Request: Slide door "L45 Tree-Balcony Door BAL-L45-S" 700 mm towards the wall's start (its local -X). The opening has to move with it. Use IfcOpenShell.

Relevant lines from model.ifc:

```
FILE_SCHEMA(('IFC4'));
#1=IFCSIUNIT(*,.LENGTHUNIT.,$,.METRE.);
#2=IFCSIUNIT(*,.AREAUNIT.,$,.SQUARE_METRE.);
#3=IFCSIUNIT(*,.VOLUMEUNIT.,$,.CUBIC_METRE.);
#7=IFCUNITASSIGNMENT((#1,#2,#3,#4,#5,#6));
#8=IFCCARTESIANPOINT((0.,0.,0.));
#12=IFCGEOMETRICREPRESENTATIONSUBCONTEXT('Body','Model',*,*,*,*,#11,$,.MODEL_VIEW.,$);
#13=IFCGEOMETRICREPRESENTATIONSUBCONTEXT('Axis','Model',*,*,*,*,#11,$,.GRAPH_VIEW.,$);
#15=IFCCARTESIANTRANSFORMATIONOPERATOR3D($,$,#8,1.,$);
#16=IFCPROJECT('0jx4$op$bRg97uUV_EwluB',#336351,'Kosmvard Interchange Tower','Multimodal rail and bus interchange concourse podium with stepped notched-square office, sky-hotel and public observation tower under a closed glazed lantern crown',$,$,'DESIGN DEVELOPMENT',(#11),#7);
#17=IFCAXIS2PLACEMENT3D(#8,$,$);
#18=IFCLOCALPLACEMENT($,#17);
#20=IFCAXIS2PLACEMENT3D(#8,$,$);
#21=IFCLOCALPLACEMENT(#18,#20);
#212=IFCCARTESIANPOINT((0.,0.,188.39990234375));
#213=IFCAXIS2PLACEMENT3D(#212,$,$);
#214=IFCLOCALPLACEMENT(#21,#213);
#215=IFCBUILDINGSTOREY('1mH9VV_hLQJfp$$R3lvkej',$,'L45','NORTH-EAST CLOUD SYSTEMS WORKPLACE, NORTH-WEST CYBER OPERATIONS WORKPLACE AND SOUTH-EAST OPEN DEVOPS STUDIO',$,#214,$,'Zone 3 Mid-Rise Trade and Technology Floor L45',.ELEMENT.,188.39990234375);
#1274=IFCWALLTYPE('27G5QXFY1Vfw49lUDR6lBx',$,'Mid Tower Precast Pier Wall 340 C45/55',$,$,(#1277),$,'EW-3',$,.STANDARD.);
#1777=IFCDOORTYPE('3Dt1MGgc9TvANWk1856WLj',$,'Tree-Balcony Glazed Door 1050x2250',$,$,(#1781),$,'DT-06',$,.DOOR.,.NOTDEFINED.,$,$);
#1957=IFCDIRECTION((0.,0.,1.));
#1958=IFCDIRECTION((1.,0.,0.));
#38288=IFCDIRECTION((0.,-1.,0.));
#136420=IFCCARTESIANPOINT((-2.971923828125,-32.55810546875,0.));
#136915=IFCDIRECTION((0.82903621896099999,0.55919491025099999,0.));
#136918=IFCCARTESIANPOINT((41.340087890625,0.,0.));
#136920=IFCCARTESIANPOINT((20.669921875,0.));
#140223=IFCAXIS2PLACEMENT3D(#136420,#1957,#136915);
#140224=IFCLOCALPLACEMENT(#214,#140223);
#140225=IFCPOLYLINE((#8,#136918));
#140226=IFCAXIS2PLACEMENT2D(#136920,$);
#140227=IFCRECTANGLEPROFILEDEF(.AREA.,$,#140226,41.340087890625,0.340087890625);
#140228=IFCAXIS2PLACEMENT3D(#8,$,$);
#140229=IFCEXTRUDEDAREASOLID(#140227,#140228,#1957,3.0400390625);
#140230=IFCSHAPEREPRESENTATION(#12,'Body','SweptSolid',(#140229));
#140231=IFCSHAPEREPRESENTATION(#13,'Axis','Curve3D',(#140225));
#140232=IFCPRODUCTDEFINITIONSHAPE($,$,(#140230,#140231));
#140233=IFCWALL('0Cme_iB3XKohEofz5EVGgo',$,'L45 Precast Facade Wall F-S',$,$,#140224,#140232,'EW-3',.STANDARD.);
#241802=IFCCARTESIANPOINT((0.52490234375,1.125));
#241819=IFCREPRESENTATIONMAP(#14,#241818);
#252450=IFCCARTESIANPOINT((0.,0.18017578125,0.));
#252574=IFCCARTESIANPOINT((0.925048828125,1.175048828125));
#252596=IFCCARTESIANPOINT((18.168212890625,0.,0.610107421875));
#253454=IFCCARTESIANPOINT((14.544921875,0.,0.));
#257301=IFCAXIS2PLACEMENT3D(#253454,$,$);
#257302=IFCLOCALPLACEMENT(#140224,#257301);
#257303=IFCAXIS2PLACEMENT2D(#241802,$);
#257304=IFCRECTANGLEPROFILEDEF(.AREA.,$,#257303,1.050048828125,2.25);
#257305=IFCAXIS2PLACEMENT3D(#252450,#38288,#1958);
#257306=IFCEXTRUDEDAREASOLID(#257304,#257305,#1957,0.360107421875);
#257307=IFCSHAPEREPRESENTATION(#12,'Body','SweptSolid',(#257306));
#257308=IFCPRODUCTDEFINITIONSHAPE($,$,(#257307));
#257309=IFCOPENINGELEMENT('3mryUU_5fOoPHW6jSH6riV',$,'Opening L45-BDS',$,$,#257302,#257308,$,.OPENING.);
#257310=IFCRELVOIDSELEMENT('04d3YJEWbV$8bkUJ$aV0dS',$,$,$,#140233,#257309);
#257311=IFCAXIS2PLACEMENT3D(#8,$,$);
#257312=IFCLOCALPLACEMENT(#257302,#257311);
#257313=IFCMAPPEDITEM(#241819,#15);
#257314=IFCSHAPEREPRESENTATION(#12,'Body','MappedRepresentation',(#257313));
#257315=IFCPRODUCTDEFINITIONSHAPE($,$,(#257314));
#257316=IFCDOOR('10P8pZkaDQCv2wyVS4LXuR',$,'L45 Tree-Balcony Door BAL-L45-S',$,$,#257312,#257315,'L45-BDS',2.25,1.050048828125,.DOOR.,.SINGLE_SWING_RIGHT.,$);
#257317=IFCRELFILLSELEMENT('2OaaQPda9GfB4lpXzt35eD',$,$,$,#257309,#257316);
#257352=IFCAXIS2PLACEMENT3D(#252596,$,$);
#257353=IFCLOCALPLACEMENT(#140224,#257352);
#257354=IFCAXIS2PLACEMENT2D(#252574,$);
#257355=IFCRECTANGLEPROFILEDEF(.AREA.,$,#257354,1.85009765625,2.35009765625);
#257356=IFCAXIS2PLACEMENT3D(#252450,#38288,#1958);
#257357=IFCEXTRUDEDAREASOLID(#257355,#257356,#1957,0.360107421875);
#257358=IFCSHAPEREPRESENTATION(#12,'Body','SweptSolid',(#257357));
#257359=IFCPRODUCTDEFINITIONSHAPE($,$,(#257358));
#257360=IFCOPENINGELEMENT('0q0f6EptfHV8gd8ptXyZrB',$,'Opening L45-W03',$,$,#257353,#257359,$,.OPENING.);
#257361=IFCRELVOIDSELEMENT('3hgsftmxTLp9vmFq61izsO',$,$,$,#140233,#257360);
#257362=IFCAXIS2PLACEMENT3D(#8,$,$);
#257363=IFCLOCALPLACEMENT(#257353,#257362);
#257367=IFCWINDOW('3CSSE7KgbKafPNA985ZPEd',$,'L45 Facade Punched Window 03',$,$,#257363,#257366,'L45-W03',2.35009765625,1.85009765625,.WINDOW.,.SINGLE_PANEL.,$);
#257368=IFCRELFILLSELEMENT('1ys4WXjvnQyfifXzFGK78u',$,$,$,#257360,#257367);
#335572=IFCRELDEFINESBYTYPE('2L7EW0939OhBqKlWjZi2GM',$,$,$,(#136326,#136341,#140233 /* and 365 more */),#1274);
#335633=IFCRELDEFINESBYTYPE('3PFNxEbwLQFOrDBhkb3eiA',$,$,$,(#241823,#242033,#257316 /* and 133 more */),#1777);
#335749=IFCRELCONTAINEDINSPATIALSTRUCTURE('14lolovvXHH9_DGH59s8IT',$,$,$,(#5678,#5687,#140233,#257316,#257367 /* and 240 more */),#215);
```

```python
import ifcopenshell
import ifcopenshell.api.geometry
import ifcopenshell.util.placement
import ifcopenshell.util.unit

model = ifcopenshell.open("model.ifc")
unit_scale = ifcopenshell.util.unit.calculate_unit_scale(model)

door = model.by_id(257316)
opening = door.FillsVoids[0].RelatingOpeningElement
wall = opening.VoidsElements[0].RelatingBuildingElement

wall_matrix = ifcopenshell.util.placement.get_local_placement(wall.ObjectPlacement)
shift = wall_matrix[:3, 0] * -0.7 / unit_scale
before = ifcopenshell.util.placement.get_local_placement(door.ObjectPlacement)[:3, 3].copy()

# The door is placed relative to its opening, so it follows when the opening moves.
matrix = ifcopenshell.util.placement.get_local_placement(opening.ObjectPlacement)
matrix[:3, 3] += shift
ifcopenshell.api.geometry.edit_object_placement(
    model, product=opening, matrix=matrix, is_si=False, should_transform_children=True
)

after = ifcopenshell.util.placement.get_local_placement(door.ObjectPlacement)[:3, 3]
print("door moved by", (after - before).round(3) + 0.0)

model.write("model-out.ifc")
```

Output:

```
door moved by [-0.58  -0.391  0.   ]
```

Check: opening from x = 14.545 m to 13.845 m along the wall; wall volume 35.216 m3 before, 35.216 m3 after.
